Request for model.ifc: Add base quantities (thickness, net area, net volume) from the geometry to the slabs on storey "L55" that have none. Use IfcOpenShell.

First a look at what the model holds.

```python
import ifcopenshell
import ifcopenshell.util.element
import ifcopenshell.util.unit

model = ifcopenshell.open("model.ifc")
print(model.schema)
for unit_type in ("LENGTHUNIT", "AREAUNIT", "VOLUMEUNIT"):
    print(unit_type, ifcopenshell.util.unit.calculate_unit_scale(model, unit_type))
storey = next(s for s in model.by_type("IfcBuildingStorey") if s.Name == "L55")
slabs = [e for e in ifcopenshell.util.element.get_decomposition(storey) if e.is_a("IfcSlab")]
for e in sorted(slabs, key=lambda e: e.id()):
    print(e.id(), e.is_a(), e.Name, list(ifcopenshell.util.element.get_psets(e, qtos_only=True)), sep=" | ")
```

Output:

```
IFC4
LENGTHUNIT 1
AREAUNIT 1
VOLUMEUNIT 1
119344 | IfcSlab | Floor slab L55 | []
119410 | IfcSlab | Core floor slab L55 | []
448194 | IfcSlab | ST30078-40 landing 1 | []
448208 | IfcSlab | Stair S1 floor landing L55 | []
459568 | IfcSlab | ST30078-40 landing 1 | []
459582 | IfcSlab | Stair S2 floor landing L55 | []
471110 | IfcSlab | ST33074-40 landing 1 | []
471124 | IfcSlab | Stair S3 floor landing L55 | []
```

```python
import ifcopenshell
import ifcopenshell.api.pset
import ifcopenshell.geom
import ifcopenshell.util.element
import ifcopenshell.util.shape
import ifcopenshell.util.unit

model = ifcopenshell.open("model.ifc")
unit_scale = ifcopenshell.util.unit.calculate_unit_scale(model)
area_scale = ifcopenshell.util.unit.calculate_unit_scale(model, "AREAUNIT")
volume_scale = ifcopenshell.util.unit.calculate_unit_scale(model, "VOLUMEUNIT")
settings = ifcopenshell.geom.settings()

storey = next(s for s in model.by_type("IfcBuildingStorey") if s.Name == "L55")
slabs = [e for e in ifcopenshell.util.element.get_decomposition(storey) if e.is_a("IfcSlab")]

for e in sorted(slabs, key=lambda e: e.id()):
    if ifcopenshell.util.element.get_psets(e, qtos_only=True, should_inherit=False):
        continue
    # Geometry comes back in metres, in the element's own axes.
    shape = ifcopenshell.geom.create_shape(settings, e)
    values = {
        "Width": ifcopenshell.util.shape.get_z(shape.geometry) / unit_scale,
        "NetArea": ifcopenshell.util.shape.get_footprint_area(shape.geometry) / area_scale,
        "NetVolume": ifcopenshell.util.shape.get_volume(shape.geometry) / volume_scale,
    }
    qto = ifcopenshell.api.pset.add_qto(model, product=e, name="Qto_SlabBaseQuantities")
    ifcopenshell.api.pset.edit_qto(model, qto=qto, properties=values)
    print(e.id(), {k: round(v, 3) for k, v in values.items()})

model.write("model_edited.ifc")
```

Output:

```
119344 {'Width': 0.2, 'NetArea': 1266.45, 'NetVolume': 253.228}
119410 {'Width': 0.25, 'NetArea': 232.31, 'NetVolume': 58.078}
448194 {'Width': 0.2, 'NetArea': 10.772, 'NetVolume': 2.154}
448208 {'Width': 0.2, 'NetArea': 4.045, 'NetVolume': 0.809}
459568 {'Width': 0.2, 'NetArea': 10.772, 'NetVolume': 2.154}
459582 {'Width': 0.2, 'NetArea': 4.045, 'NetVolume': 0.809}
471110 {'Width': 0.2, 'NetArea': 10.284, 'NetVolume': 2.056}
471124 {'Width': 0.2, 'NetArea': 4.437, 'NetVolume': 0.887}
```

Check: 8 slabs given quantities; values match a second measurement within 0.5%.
